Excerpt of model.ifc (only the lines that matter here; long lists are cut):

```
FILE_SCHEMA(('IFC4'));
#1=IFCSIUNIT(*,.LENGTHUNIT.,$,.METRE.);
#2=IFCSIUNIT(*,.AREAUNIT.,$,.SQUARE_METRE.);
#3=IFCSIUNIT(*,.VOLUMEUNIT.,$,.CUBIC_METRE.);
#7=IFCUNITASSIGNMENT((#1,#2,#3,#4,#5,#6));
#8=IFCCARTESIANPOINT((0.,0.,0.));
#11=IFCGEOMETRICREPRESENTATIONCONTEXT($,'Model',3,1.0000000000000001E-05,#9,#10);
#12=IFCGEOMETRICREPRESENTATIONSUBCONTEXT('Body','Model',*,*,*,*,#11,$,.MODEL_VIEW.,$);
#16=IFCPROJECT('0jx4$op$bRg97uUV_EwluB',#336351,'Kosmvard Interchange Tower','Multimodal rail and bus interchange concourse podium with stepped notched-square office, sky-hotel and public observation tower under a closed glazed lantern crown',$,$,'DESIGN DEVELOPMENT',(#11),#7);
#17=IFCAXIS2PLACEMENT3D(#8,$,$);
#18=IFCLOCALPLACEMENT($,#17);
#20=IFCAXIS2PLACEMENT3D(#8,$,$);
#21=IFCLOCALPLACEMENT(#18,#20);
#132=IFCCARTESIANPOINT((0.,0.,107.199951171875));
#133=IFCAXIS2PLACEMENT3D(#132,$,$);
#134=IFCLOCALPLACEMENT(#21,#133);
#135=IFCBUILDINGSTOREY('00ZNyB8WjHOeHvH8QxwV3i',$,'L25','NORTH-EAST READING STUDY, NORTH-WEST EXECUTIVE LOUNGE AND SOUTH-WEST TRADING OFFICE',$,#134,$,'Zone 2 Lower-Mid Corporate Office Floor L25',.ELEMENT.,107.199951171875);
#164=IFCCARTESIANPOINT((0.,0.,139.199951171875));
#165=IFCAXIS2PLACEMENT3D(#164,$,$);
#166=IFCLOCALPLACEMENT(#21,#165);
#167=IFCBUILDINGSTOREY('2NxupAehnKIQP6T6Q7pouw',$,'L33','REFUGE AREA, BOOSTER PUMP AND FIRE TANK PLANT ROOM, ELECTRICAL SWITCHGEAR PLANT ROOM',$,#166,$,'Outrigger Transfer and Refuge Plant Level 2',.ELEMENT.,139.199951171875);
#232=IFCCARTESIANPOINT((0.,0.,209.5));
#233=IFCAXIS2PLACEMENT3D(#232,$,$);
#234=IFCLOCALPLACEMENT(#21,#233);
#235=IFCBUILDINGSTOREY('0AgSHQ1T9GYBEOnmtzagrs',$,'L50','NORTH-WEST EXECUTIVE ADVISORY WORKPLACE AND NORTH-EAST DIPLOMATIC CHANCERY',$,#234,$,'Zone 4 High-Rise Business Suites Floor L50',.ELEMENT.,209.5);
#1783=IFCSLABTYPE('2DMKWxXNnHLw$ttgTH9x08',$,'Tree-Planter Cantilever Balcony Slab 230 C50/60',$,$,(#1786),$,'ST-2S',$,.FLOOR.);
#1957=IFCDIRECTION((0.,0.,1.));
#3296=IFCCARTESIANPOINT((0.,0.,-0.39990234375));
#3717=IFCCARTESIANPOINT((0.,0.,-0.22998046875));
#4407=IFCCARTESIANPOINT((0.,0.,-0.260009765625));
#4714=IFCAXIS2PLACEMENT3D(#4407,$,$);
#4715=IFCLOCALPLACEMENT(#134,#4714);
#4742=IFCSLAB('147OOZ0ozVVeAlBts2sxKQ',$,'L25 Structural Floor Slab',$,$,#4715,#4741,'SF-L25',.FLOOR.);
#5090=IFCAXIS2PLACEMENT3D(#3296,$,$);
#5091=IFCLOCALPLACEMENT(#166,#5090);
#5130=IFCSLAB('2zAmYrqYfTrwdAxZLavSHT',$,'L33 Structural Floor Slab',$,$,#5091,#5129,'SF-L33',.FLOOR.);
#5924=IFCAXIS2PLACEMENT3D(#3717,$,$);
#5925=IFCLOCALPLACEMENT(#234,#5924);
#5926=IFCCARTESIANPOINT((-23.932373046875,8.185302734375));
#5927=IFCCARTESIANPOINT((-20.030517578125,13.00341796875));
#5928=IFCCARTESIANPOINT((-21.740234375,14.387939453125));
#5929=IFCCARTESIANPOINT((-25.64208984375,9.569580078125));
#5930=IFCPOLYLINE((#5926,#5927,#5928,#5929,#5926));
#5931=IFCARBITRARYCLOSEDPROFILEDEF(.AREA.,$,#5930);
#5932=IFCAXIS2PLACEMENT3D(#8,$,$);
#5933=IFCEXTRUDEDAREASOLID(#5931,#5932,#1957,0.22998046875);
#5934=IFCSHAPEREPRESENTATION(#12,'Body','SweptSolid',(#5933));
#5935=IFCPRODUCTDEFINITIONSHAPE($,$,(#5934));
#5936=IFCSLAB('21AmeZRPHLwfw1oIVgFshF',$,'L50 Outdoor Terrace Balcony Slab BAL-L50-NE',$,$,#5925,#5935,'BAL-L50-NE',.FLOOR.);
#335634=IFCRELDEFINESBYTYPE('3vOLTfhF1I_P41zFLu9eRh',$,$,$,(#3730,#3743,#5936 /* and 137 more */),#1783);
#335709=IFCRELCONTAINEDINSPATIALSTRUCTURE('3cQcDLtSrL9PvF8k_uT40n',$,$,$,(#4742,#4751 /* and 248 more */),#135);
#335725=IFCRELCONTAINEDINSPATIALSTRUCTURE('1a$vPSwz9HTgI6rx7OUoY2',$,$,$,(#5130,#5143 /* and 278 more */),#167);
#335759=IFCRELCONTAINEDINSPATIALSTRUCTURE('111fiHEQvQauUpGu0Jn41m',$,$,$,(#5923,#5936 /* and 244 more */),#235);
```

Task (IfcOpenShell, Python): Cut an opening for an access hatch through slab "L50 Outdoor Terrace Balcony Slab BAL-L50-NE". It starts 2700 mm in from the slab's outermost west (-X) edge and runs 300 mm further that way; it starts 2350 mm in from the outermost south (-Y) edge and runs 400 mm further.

```python
import numpy as np
import ifcopenshell
import ifcopenshell.api.feature
import ifcopenshell.api.geometry
import ifcopenshell.api.root
import ifcopenshell.geom
import ifcopenshell.util.placement
import ifcopenshell.util.representation
import ifcopenshell.util.shape
import ifcopenshell.util.unit

model = ifcopenshell.open("model.ifc")
unit_scale = ifcopenshell.util.unit.calculate_unit_scale(model)
settings = ifcopenshell.geom.settings()


def volume(element):
    """Net volume in cubic metres, openings subtracted."""
    shape = ifcopenshell.geom.create_shape(settings, element)
    return ifcopenshell.util.shape.get_volume(shape.geometry)


slab = model.by_guid("21AmeZRPHLwfw1oIVgFshF")
before = volume(slab)

# Extent in the slab's own axes, in metres. The edges named are its -X and -Y sides.
slab_shape = ifcopenshell.geom.create_shape(settings, slab)
vertices = ifcopenshell.util.shape.get_vertices(slab_shape.geometry)
x_min, y_min, bottom = vertices.min(axis=0)
top = vertices[:, 2].max()

opening = ifcopenshell.api.root.create_entity(model, ifc_class="IfcOpeningElement", name="Access hatch opening", predefined_type="OPENING")
context = ifcopenshell.util.representation.get_context(model, "Model", "Body", "MODEL_VIEW")
width, depth = 0.3, 0.4
outline = [(0.0, 0.0), (width, 0.0), (width, depth), (0.0, depth), (0.0, 0.0)]
# Overshoot both faces by 50 mm so the cut is clean.
shape = ifcopenshell.api.geometry.add_slab_representation(
    model, context=context, depth=top - bottom + 0.1, polyline=outline
)
ifcopenshell.api.geometry.assign_representation(model, product=opening, representation=shape)

matrix = ifcopenshell.util.placement.get_local_placement(slab.ObjectPlacement)
matrix[:, 3] = matrix @ np.append(np.array([x_min + 2.7, y_min + 2.35, bottom - 0.05]) / unit_scale, 1.0)
ifcopenshell.api.geometry.edit_object_placement(model, product=opening, matrix=matrix, is_si=False)
ifcopenshell.api.feature.add_feature(model, feature=opening, element=slab)

after = volume(slab)

print(f"slab volume {before:.3f} -> {after:.3f} m3")

model.write("model_v2.ifc")
```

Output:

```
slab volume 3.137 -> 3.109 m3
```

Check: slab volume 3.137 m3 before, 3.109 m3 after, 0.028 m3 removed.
